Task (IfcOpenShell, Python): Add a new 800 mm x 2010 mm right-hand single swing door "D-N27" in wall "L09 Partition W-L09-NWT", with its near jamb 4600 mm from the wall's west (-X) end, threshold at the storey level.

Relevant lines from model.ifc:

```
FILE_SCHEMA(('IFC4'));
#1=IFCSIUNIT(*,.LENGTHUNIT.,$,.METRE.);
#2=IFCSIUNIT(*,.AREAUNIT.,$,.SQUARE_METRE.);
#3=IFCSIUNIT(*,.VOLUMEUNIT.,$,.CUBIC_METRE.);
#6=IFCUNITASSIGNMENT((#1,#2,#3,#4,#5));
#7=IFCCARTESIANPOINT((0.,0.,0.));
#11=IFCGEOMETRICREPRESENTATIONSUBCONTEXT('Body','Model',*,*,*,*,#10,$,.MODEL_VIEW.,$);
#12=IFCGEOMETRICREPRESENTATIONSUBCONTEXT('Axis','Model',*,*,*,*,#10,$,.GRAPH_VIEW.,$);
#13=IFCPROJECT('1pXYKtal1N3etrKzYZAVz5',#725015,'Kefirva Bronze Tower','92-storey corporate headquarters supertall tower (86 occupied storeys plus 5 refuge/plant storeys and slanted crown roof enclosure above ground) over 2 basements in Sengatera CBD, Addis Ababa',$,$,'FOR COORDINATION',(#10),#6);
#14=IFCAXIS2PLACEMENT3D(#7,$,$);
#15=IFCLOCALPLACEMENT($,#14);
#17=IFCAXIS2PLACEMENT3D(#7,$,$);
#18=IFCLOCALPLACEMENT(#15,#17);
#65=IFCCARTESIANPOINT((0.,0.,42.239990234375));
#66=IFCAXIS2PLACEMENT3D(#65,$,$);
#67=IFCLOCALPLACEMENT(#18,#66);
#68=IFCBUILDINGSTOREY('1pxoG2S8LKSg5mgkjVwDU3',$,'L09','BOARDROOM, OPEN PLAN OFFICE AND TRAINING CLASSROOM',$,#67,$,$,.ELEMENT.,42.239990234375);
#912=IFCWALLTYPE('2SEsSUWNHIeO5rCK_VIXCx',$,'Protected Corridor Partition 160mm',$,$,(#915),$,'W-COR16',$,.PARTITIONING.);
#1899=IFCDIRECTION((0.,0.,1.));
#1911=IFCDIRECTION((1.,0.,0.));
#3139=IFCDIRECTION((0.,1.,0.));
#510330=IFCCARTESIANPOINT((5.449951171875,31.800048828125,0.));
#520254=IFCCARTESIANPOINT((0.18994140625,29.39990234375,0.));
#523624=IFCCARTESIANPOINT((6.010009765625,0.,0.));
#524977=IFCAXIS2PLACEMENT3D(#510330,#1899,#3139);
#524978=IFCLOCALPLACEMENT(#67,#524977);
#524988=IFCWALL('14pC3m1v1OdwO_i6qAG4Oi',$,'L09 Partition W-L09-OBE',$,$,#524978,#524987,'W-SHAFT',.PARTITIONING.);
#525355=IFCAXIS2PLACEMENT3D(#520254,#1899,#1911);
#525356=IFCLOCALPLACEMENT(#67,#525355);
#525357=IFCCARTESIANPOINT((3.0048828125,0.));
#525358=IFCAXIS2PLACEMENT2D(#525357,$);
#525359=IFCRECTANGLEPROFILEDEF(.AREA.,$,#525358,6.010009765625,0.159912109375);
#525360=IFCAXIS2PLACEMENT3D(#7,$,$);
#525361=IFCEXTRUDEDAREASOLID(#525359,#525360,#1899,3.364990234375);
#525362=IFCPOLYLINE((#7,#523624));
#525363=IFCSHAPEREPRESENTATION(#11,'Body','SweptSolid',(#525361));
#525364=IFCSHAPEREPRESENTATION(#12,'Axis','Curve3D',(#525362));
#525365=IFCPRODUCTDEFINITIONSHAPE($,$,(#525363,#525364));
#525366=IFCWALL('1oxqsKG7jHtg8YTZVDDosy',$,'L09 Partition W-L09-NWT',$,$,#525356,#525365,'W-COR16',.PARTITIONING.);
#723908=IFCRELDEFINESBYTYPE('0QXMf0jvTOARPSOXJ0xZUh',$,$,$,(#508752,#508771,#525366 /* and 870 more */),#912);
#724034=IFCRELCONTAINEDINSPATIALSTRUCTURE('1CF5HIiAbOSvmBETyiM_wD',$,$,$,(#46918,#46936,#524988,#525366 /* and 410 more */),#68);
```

```python
import numpy as np
import ifcopenshell
import ifcopenshell.api.feature
import ifcopenshell.api.geometry
import ifcopenshell.api.root
import ifcopenshell.api.spatial
import ifcopenshell.geom
import ifcopenshell.util.element
import ifcopenshell.util.placement
import ifcopenshell.util.representation
import ifcopenshell.util.shape
import ifcopenshell.util.unit

model = ifcopenshell.open("model.ifc")
unit_scale = ifcopenshell.util.unit.calculate_unit_scale(model)
settings = ifcopenshell.geom.settings()


def volume(element):
    """Net volume in cubic metres, openings subtracted."""
    shape = ifcopenshell.geom.create_shape(settings, element)
    return ifcopenshell.util.shape.get_volume(shape.geometry)


wall = model.by_guid("1oxqsKG7jHtg8YTZVDDosy")
storey = ifcopenshell.util.element.get_container(wall, ifc_class="IfcBuildingStorey")
context = ifcopenshell.util.representation.get_context(model, "Model", "Body", "MODEL_VIEW")
before = volume(wall)

width, height, from_end, sill = 0.8, 2.01, 4.6, 0.0  # metres

# The wall runs along its own X axis, and the end named is its -X end.
wall_shape = ifcopenshell.geom.create_shape(settings, wall)
x, y, z = ifcopenshell.util.shape.get_vertices(wall_shape.geometry).T
start = x.min() + from_end
face, thickness = float(y.min()), float(y.max() - y.min())
wall_matrix = ifcopenshell.util.placement.get_local_placement(wall.ObjectPlacement)
level = ifcopenshell.util.placement.get_local_placement(storey.ObjectPlacement)[2, 3]


def in_wall(x, y):
    """Placement at x, y metres in the wall's axes, at sill height."""
    matrix = wall_matrix.copy()
    matrix[:, 3] = wall_matrix @ np.array([x / unit_scale, y / unit_scale, 0.0, 1.0])
    matrix[2, 3] = level + sill / unit_scale
    return matrix


# Opening: a box that overshoots both wall faces by 50 mm.
opening = ifcopenshell.api.root.create_entity(model, ifc_class="IfcOpeningElement", predefined_type="OPENING")
box = ifcopenshell.api.geometry.add_wall_representation(
    model, context=context, length=width, height=height, thickness=thickness + 0.1
)
ifcopenshell.api.geometry.assign_representation(model, product=opening, representation=box)
ifcopenshell.api.geometry.edit_object_placement(model, product=opening, matrix=in_wall(start, face - 0.05), is_si=False)
ifcopenshell.api.feature.add_feature(model, feature=opening, element=wall)

door = ifcopenshell.api.root.create_entity(model, ifc_class="IfcDoor", name="D-N27", predefined_type="DOOR")
door.OverallWidth, door.OverallHeight = width / unit_scale, height / unit_scale
door.OperationType = "SINGLE_SWING_RIGHT"
body = ifcopenshell.api.geometry.add_door_representation(
    model,
    context=context,
    overall_width=door.OverallWidth,
    overall_height=door.OverallHeight,
    operation_type="SINGLE_SWING_RIGHT",
    lining_properties={"LiningDepth": thickness / unit_scale, "ThresholdDepth": thickness / unit_scale},
)
ifcopenshell.api.geometry.assign_representation(model, product=door, representation=body)
ifcopenshell.api.spatial.assign_container(model, products=[door], relating_structure=storey)
ifcopenshell.api.feature.add_filling(model, opening=opening, element=door)

# The lining spans the wall, so the door starts at the wall face.
ifcopenshell.api.geometry.edit_object_placement(model, product=door, matrix=in_wall(start, face), is_si=False)

after = volume(wall)

print(f"wall volume {before:.3f} -> {after:.3f} m3")

model.write("model_updated.ifc")
```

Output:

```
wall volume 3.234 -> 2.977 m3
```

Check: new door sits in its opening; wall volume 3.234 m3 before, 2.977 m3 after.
